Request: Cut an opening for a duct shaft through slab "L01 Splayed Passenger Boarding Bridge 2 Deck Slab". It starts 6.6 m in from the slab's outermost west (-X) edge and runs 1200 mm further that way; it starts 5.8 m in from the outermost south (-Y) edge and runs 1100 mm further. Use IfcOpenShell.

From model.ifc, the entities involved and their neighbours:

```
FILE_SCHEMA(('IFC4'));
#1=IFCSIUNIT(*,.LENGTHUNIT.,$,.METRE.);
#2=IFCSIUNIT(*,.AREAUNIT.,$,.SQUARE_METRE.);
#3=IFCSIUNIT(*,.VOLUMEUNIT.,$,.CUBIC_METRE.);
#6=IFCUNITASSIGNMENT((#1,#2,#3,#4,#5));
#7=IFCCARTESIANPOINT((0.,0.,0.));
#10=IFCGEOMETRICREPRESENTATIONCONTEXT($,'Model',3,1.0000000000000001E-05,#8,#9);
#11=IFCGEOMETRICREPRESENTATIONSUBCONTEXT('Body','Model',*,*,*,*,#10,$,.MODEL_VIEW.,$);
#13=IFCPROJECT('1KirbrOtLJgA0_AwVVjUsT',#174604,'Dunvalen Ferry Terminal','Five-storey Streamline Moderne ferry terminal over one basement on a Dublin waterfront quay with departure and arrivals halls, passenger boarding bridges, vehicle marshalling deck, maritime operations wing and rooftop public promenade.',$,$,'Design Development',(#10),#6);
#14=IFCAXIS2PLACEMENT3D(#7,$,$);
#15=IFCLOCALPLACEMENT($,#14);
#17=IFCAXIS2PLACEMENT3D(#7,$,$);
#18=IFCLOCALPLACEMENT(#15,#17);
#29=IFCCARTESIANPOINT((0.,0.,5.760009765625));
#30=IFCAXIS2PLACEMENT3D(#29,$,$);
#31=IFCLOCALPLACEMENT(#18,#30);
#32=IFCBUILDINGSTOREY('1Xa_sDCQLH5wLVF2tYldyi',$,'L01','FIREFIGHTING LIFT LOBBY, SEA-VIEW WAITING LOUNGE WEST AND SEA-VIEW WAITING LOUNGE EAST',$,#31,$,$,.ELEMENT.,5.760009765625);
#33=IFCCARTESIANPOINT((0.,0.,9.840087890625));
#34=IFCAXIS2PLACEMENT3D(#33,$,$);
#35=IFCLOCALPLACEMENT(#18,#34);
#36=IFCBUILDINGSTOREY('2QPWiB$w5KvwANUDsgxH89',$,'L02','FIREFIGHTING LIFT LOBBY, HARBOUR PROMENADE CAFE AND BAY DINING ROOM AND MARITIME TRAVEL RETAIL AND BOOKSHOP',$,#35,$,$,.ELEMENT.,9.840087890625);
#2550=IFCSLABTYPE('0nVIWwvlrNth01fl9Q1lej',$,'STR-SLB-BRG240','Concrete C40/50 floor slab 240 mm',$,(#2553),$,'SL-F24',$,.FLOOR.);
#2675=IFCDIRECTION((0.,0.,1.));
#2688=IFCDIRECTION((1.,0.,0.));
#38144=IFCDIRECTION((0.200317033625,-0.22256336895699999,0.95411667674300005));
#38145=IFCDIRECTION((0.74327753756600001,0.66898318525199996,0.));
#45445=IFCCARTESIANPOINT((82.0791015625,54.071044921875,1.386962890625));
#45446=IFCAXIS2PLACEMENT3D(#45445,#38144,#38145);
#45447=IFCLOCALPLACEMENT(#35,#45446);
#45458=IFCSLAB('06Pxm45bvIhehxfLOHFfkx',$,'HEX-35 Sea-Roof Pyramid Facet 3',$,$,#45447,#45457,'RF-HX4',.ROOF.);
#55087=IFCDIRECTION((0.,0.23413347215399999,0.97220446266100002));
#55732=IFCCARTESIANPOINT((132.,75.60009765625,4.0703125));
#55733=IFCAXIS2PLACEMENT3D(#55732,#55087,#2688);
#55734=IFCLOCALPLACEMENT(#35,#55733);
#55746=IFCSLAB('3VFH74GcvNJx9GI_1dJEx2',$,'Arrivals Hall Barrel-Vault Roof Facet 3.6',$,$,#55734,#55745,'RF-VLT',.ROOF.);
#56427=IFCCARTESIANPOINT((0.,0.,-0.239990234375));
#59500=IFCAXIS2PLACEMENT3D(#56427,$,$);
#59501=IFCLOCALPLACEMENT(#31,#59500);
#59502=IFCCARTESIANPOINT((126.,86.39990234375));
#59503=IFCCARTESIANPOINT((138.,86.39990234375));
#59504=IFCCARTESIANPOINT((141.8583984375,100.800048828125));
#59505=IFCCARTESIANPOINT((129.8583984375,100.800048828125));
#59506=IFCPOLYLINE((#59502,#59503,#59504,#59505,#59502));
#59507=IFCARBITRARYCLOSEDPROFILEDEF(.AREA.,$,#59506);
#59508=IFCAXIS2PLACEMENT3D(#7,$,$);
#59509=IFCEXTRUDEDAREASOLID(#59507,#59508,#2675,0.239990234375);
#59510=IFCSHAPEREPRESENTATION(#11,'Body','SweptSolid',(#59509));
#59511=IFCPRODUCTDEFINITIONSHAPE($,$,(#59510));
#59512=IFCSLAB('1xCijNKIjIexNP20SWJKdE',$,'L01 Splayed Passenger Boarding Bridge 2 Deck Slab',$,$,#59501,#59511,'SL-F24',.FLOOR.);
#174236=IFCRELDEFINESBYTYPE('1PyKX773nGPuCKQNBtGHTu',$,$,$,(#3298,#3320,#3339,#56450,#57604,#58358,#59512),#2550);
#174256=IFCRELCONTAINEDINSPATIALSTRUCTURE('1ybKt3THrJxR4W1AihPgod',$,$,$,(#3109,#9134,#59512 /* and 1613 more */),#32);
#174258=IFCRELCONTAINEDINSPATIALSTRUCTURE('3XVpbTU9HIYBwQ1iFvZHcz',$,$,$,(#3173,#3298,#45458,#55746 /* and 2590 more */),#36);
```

```python
import numpy as np
import ifcopenshell
import ifcopenshell.api.feature
import ifcopenshell.api.geometry
import ifcopenshell.api.root
import ifcopenshell.geom
import ifcopenshell.util.placement
import ifcopenshell.util.representation
import ifcopenshell.util.shape
import ifcopenshell.util.unit

model = ifcopenshell.open("model.ifc")
unit_scale = ifcopenshell.util.unit.calculate_unit_scale(model)
settings = ifcopenshell.geom.settings()


def volume(element):
    """Net volume in cubic metres, openings subtracted."""
    shape = ifcopenshell.geom.create_shape(settings, element)
    return ifcopenshell.util.shape.get_volume(shape.geometry)


slab = model.by_guid("1xCijNKIjIexNP20SWJKdE")
before = volume(slab)

# Extent in the slab's own axes, in metres. The edges named are its -X and -Y sides.
slab_shape = ifcopenshell.geom.create_shape(settings, slab)
vertices = ifcopenshell.util.shape.get_vertices(slab_shape.geometry)
x_min, y_min, bottom = vertices.min(axis=0)
top = vertices[:, 2].max()

opening = ifcopenshell.api.root.create_entity(model, ifc_class="IfcOpeningElement", name="Duct shaft opening", predefined_type="OPENING")
context = ifcopenshell.util.representation.get_context(model, "Model", "Body", "MODEL_VIEW")
width, depth = 1.2, 1.1
outline = [(0.0, 0.0), (width, 0.0), (width, depth), (0.0, depth), (0.0, 0.0)]
# Overshoot both faces by 50 mm so the cut is clean.
shape = ifcopenshell.api.geometry.add_slab_representation(
    model, context=context, depth=top - bottom + 0.1, polyline=outline
)
ifcopenshell.api.geometry.assign_representation(model, product=opening, representation=shape)

matrix = ifcopenshell.util.placement.get_local_placement(slab.ObjectPlacement)
matrix[:, 3] = matrix @ np.append(np.array([x_min + 6.6, y_min + 5.8, bottom - 0.05]) / unit_scale, 1.0)
ifcopenshell.api.geometry.edit_object_placement(model, product=opening, matrix=matrix, is_si=False)
ifcopenshell.api.feature.add_feature(model, feature=opening, element=slab)

after = volume(slab)

print(f"slab volume {before:.3f} -> {after:.3f} m3")

model.write("model_rev.ifc")
```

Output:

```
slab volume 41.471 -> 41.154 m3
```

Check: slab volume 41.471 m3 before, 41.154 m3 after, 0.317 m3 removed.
